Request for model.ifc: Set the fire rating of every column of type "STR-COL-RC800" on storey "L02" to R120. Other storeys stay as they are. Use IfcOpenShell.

First a look at what the model holds.

```python
import ifcopenshell
import ifcopenshell.util.element

model = ifcopenshell.open("model.ifc")
print(model.schema)
storey = next(s for s in model.by_type("IfcBuildingStorey") if s.Name == "L02")
columns = [e for e in ifcopenshell.util.element.get_decomposition(storey) if e.is_a("IfcColumn")]
seen = {}
for e in columns:
    element_type = ifcopenshell.util.element.get_type(e)
    key = (element_type.Name if element_type != e and element_type else None, ifcopenshell.util.element.get_pset(e, "Pset_ColumnCommon", "FireRating"))
    seen[key] = seen.get(key, 0) + 1
for (name, value), count in sorted(seen.items(), key=str):
    print(count, "x", name, "|", value)
```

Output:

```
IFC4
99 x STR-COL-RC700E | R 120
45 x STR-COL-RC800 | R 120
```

```python
import ifcopenshell
import ifcopenshell.api.pset
import ifcopenshell.util.element

model = ifcopenshell.open("model.ifc")

storey = next(s for s in model.by_type("IfcBuildingStorey") if s.Name == "L02")
columns = [e for e in ifcopenshell.util.element.get_decomposition(storey) if e.is_a("IfcColumn")]

count = 0
for e in columns:
    element_type = ifcopenshell.util.element.get_type(e)
    if element_type in (None, e) or element_type.Name != "STR-COL-RC800":
        continue
    # add_pset returns the element's existing set when there is one.
    pset = ifcopenshell.api.pset.add_pset(model, product=e, name="Pset_ColumnCommon")
    ifcopenshell.api.pset.edit_pset(model, pset=pset, properties={"FireRating": "R120"})
    count += 1

print(count, "columns updated")

model.write("model_rev.ifc")
```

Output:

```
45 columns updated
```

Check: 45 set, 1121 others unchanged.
